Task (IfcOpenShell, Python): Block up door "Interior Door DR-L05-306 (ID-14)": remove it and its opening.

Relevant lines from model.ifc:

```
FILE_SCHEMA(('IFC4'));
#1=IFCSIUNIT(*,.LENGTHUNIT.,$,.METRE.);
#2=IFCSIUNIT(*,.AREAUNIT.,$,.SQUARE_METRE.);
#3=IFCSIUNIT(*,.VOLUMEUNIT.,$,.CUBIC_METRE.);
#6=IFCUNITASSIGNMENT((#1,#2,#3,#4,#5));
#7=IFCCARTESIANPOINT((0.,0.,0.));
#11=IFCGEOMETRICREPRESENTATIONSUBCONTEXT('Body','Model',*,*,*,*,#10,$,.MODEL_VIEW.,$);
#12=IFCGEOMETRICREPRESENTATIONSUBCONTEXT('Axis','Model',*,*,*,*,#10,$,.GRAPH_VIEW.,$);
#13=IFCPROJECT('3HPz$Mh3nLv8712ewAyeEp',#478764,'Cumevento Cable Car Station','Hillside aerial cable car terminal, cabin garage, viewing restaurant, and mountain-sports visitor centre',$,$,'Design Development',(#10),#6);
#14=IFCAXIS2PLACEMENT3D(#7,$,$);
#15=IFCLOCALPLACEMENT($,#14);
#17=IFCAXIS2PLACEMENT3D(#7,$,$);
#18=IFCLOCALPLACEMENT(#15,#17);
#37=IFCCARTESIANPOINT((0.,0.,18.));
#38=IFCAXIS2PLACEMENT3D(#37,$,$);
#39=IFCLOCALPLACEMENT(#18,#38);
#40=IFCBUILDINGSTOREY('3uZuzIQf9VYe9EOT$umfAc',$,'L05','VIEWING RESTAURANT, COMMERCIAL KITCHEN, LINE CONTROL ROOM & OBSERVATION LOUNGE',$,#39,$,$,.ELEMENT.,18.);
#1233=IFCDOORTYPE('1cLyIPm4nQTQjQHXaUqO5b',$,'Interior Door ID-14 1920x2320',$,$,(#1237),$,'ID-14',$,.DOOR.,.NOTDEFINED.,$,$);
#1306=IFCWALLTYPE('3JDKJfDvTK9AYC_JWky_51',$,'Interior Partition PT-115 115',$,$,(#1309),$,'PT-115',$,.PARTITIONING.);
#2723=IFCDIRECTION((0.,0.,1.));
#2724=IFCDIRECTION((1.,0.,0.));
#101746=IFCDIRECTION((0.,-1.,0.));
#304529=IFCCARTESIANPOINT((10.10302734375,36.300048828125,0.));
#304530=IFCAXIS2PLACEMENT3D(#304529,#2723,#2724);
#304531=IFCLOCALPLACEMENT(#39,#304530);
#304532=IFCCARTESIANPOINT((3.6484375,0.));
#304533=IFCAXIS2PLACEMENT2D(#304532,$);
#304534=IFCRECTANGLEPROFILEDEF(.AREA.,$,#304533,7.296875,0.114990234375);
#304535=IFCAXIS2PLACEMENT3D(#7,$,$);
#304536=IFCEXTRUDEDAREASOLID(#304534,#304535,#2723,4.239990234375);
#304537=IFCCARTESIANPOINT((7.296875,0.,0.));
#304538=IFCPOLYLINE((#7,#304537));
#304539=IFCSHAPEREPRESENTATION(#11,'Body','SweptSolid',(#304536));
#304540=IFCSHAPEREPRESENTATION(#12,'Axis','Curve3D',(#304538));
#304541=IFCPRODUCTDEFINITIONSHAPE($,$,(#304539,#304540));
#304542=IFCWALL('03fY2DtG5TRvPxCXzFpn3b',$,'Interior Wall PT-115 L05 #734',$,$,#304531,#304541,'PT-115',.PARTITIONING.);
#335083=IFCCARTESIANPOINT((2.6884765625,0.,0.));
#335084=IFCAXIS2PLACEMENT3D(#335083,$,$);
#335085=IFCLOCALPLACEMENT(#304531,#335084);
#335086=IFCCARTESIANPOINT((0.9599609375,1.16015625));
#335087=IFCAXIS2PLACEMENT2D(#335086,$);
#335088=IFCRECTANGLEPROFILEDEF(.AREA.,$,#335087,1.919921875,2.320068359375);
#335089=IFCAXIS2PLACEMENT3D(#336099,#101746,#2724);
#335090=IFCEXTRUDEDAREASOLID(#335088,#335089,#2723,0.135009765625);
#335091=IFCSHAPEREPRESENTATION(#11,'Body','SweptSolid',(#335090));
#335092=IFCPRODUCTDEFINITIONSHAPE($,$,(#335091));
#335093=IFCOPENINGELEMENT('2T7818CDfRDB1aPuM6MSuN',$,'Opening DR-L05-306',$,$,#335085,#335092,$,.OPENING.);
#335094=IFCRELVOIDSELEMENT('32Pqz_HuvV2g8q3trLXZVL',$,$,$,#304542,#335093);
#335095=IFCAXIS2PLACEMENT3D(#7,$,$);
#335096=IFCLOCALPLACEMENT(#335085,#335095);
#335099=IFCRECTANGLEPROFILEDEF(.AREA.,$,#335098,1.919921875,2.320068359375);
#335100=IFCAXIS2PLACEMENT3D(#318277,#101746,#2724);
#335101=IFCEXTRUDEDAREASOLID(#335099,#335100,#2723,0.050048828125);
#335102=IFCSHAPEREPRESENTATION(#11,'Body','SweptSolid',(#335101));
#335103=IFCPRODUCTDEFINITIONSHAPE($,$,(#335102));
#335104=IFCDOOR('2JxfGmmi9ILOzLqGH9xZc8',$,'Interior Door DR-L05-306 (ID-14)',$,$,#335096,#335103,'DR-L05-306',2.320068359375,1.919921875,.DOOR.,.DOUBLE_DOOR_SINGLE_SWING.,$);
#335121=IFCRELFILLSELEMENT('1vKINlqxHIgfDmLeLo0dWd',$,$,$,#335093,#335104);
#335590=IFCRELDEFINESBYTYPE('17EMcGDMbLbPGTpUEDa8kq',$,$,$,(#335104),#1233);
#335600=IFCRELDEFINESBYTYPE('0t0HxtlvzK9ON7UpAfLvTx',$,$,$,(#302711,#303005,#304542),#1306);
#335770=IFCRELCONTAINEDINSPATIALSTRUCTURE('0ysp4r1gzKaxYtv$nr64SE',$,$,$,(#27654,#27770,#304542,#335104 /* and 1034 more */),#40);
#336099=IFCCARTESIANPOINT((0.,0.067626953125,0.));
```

```python
import ifcopenshell
import ifcopenshell.api.feature
import ifcopenshell.api.root
import ifcopenshell.geom
import ifcopenshell.util.shape

model = ifcopenshell.open("model.ifc")
settings = ifcopenshell.geom.settings()


def volume(element):
    """Net volume in cubic metres, openings subtracted."""
    shape = ifcopenshell.geom.create_shape(settings, element)
    return ifcopenshell.util.shape.get_volume(shape.geometry)


door = model.by_id(335104)
opening = door.FillsVoids[0].RelatingOpeningElement
wall = opening.VoidsElements[0].RelatingBuildingElement
before = volume(wall)

ifcopenshell.api.root.remove_product(model, product=door)
ifcopenshell.api.feature.remove_feature(model, feature=opening)

after = volume(wall)

print(f"wall volume {before:.3f} -> {after:.3f} m3")

model.write("model_updated.ifc")
```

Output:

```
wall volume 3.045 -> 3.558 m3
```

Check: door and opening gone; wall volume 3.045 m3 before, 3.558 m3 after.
